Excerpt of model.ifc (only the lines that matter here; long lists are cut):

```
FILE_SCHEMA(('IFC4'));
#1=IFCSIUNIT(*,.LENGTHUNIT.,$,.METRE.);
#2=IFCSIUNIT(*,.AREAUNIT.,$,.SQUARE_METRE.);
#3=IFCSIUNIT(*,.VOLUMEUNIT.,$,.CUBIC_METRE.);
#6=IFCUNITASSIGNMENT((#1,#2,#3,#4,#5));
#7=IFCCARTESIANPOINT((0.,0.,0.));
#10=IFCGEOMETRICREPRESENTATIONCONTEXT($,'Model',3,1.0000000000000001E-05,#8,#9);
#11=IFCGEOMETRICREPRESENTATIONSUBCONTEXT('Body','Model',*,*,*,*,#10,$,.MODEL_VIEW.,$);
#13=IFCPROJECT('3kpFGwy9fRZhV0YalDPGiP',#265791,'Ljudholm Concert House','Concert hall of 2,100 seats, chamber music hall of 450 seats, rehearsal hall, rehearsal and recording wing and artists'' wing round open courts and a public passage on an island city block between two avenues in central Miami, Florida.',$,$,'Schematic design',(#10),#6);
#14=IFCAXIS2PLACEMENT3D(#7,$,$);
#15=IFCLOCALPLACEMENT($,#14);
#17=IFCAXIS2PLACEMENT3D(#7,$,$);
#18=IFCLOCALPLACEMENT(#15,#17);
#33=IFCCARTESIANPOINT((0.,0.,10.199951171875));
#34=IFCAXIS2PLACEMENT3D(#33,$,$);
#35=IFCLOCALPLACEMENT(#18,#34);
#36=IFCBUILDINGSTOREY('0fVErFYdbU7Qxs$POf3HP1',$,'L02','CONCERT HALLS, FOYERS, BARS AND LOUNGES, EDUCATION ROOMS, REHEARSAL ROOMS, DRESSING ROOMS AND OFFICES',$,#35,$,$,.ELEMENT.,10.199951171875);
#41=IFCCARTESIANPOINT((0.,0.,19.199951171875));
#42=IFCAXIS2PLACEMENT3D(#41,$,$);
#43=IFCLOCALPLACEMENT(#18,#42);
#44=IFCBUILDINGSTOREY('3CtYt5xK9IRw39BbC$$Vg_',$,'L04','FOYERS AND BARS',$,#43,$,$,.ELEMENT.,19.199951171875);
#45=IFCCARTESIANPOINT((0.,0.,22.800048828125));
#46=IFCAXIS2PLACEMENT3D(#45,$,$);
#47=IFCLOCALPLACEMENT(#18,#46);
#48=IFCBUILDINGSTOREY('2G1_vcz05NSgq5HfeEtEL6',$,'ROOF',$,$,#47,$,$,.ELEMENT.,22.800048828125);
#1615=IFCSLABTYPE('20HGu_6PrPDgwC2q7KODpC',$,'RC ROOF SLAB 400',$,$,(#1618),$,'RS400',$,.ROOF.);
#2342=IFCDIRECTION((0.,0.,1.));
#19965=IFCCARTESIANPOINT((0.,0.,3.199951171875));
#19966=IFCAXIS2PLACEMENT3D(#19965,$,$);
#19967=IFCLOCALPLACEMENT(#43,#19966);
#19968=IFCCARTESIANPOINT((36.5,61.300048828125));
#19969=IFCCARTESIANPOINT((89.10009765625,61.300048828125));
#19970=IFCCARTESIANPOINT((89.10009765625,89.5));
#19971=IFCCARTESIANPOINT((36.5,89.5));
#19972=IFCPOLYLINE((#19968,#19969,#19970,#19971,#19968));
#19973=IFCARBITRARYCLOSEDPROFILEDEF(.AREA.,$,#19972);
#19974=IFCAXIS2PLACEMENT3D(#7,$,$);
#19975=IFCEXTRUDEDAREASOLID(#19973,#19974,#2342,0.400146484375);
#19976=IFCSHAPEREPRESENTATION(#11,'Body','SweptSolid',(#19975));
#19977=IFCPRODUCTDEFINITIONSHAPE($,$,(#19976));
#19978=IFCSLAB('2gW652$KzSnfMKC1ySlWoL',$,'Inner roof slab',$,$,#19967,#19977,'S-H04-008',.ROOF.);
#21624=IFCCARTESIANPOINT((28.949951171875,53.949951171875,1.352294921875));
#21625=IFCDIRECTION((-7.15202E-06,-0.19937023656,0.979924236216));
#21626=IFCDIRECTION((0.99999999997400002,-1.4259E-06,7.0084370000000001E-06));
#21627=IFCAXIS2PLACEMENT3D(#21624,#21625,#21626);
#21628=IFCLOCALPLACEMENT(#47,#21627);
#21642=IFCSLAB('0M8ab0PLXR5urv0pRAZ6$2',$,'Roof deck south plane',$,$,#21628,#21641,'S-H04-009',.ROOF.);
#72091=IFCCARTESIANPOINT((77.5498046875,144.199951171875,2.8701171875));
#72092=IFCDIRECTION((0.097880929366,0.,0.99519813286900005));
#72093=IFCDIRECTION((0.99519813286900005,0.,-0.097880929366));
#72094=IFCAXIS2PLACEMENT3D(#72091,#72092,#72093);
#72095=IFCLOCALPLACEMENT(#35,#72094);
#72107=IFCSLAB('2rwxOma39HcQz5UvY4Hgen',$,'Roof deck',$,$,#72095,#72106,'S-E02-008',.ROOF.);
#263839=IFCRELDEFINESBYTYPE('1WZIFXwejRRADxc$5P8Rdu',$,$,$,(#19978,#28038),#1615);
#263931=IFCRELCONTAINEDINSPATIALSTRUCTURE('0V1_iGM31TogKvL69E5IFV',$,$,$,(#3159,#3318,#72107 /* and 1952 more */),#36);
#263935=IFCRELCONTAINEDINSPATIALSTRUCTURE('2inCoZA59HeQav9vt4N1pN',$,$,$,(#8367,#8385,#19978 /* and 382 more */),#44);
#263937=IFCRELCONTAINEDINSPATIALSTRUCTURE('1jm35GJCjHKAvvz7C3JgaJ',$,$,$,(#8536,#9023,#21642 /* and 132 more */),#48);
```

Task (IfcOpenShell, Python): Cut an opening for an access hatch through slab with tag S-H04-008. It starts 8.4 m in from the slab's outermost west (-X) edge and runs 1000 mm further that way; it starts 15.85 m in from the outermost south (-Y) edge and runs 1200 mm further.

```python
import numpy as np
import ifcopenshell
import ifcopenshell.api.feature
import ifcopenshell.api.geometry
import ifcopenshell.api.root
import ifcopenshell.geom
import ifcopenshell.util.placement
import ifcopenshell.util.representation
import ifcopenshell.util.shape
import ifcopenshell.util.unit

model = ifcopenshell.open("model.ifc")
unit_scale = ifcopenshell.util.unit.calculate_unit_scale(model)
settings = ifcopenshell.geom.settings()


def volume(element):
    """Net volume in cubic metres, openings subtracted."""
    shape = ifcopenshell.geom.create_shape(settings, element)
    return ifcopenshell.util.shape.get_volume(shape.geometry)


slab = model.by_guid("2gW652$KzSnfMKC1ySlWoL")
before = volume(slab)

# Extent in the slab's own axes, in metres. The edges named are its -X and -Y sides.
slab_shape = ifcopenshell.geom.create_shape(settings, slab)
vertices = ifcopenshell.util.shape.get_vertices(slab_shape.geometry)
x_min, y_min, bottom = vertices.min(axis=0)
top = vertices[:, 2].max()

opening = ifcopenshell.api.root.create_entity(model, ifc_class="IfcOpeningElement", name="Access hatch opening", predefined_type="OPENING")
context = ifcopenshell.util.representation.get_context(model, "Model", "Body", "MODEL_VIEW")
width, depth = 1, 1.2
outline = [(0.0, 0.0), (width, 0.0), (width, depth), (0.0, depth), (0.0, 0.0)]
# Overshoot both faces by 50 mm so the cut is clean.
shape = ifcopenshell.api.geometry.add_slab_representation(
    model, context=context, depth=top - bottom + 0.1, polyline=outline
)
ifcopenshell.api.geometry.assign_representation(model, product=opening, representation=shape)

matrix = ifcopenshell.util.placement.get_local_placement(slab.ObjectPlacement)
matrix[:, 3] = matrix @ np.append(np.array([x_min + 8.4, y_min + 15.85, bottom - 0.05]) / unit_scale, 1.0)
ifcopenshell.api.geometry.edit_object_placement(model, product=opening, matrix=matrix, is_si=False)
ifcopenshell.api.feature.add_feature(model, feature=opening, element=slab)

after = volume(slab)

print(f"slab volume {before:.3f} -> {after:.3f} m3")

model.write("model_updated.ifc")
```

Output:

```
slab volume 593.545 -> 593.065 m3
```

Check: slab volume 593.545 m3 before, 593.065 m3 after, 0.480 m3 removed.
